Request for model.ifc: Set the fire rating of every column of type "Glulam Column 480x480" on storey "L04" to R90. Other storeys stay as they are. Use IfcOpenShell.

First a look at what the model holds.

```python
import ifcopenshell
import ifcopenshell.util.element

model = ifcopenshell.open("model.ifc")
print(model.schema)
storey = next(s for s in model.by_type("IfcBuildingStorey") if s.Name == "L04")
columns = [e for e in ifcopenshell.util.element.get_decomposition(storey) if e.is_a("IfcColumn")]
seen = {}
for e in columns:
    element_type = ifcopenshell.util.element.get_type(e)
    key = (element_type.Name if element_type != e and element_type else None, ifcopenshell.util.element.get_pset(e, "Pset_ColumnCommon", "FireRating"))
    seen[key] = seen.get(key, 0) + 1
for (name, value), count in sorted(seen.items(), key=str):
    print(count, "x", name, "|", value)
```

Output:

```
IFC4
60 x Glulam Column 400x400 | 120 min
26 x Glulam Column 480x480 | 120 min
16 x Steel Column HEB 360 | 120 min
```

```python
import ifcopenshell
import ifcopenshell.api.pset
import ifcopenshell.util.element

model = ifcopenshell.open("model.ifc")

storey = next(s for s in model.by_type("IfcBuildingStorey") if s.Name == "L04")
columns = [e for e in ifcopenshell.util.element.get_decomposition(storey) if e.is_a("IfcColumn")]

count = 0
for e in columns:
    element_type = ifcopenshell.util.element.get_type(e)
    if element_type in (None, e) or element_type.Name != "Glulam Column 480x480":
        continue
    # add_pset returns the element's existing set when there is one.
    pset = ifcopenshell.api.pset.add_pset(model, product=e, name="Pset_ColumnCommon")
    ifcopenshell.api.pset.edit_pset(model, pset=pset, properties={"FireRating": "R90"})
    count += 1

print(count, "columns updated")

model.write("model_updated.ifc")
```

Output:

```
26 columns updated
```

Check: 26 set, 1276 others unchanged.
